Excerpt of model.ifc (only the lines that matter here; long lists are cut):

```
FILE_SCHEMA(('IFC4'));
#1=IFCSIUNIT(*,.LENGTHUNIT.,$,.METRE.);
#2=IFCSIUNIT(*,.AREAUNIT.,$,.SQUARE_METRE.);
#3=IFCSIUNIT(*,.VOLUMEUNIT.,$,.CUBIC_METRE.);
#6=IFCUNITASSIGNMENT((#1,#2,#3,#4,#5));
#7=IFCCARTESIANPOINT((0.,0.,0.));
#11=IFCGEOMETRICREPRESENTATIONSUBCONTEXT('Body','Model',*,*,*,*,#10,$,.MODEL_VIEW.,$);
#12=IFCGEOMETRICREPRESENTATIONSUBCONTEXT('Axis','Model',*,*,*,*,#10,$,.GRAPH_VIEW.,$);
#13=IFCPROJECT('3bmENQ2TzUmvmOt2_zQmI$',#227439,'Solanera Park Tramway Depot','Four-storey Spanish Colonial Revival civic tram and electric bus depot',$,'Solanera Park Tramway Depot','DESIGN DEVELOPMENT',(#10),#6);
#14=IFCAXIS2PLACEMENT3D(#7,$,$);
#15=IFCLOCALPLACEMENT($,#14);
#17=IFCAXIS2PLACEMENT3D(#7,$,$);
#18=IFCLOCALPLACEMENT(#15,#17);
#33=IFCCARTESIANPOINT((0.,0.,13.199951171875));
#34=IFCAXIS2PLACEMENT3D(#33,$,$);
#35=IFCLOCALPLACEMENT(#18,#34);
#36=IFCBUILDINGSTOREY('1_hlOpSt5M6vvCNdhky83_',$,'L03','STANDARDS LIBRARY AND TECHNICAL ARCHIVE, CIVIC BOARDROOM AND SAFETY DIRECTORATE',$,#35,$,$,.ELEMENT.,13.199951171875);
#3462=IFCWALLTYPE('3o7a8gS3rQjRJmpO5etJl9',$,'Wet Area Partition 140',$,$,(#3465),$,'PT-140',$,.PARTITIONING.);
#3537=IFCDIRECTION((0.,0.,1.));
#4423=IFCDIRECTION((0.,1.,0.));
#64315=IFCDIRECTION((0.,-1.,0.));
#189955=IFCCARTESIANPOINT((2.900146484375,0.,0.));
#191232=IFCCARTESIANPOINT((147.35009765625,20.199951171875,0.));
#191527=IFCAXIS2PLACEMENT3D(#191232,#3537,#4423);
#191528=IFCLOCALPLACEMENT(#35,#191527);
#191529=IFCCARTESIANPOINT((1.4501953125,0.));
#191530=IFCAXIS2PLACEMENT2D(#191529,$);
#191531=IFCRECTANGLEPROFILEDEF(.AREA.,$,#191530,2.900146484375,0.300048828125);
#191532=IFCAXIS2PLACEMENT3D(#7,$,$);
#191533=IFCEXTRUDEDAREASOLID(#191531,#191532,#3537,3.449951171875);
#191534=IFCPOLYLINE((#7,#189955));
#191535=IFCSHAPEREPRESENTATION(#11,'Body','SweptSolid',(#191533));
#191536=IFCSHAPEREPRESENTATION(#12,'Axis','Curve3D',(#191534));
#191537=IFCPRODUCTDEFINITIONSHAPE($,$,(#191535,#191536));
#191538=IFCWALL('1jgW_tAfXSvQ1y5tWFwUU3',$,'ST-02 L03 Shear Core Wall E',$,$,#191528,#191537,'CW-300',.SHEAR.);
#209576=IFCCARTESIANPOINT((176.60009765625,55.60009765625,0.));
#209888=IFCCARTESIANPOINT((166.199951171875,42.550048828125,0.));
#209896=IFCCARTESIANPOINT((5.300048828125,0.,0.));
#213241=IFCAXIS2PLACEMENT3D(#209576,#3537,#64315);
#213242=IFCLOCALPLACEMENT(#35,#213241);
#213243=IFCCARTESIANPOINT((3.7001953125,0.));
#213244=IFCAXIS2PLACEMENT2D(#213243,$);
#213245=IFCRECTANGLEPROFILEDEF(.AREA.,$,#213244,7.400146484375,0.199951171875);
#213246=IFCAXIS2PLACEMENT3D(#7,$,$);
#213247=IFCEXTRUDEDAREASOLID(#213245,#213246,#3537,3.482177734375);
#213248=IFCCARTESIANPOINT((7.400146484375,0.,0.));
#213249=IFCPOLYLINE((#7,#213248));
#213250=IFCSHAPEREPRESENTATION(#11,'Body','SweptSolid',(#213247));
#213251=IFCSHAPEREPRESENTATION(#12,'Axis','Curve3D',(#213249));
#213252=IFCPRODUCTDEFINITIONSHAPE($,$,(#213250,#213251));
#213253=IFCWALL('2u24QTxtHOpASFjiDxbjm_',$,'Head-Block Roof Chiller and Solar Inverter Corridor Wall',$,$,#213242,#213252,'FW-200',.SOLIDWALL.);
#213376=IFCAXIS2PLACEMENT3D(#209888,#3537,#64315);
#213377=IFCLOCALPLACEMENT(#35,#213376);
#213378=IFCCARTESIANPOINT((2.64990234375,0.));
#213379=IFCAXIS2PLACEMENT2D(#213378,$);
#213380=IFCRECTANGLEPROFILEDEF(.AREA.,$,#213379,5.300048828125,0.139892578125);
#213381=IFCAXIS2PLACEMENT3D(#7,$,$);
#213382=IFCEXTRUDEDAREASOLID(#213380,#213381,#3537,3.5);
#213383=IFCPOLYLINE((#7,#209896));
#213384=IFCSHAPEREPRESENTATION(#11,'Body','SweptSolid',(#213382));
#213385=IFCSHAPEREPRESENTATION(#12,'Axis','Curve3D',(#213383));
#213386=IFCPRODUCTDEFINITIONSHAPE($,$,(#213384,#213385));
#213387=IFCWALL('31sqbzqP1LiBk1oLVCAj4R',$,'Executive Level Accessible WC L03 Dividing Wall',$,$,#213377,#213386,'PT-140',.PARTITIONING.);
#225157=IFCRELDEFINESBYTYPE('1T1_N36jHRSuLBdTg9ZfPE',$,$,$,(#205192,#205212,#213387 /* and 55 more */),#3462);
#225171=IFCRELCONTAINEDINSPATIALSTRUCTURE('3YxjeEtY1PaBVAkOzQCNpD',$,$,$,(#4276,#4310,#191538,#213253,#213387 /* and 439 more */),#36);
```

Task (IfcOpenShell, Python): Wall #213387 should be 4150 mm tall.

```python
import ifcopenshell
import ifcopenshell.geom
import ifcopenshell.util.representation
import ifcopenshell.util.shape
import ifcopenshell.util.unit

model = ifcopenshell.open("model.ifc")
unit_scale = ifcopenshell.util.unit.calculate_unit_scale(model)
settings = ifcopenshell.geom.settings()


def volume(element):
    """Net volume in cubic metres, openings subtracted."""
    shape = ifcopenshell.geom.create_shape(settings, element)
    return ifcopenshell.util.shape.get_volume(shape.geometry)


wall = model.by_guid("31sqbzqP1LiBk1oLVCAj4R")
before = volume(wall)

body = ifcopenshell.util.representation.get_representation(wall, "Model", "Body")
solid = body.Items[0]
old_height = solid.Depth
solid.Depth = 4.15 / unit_scale
after = volume(wall)

print(f"height {old_height:g} -> {solid.Depth:g}, volume {before:.3f} -> {after:.3f} m3")

model.write("model_rev.ifc")
```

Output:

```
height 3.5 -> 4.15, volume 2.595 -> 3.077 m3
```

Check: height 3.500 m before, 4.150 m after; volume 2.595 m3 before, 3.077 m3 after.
